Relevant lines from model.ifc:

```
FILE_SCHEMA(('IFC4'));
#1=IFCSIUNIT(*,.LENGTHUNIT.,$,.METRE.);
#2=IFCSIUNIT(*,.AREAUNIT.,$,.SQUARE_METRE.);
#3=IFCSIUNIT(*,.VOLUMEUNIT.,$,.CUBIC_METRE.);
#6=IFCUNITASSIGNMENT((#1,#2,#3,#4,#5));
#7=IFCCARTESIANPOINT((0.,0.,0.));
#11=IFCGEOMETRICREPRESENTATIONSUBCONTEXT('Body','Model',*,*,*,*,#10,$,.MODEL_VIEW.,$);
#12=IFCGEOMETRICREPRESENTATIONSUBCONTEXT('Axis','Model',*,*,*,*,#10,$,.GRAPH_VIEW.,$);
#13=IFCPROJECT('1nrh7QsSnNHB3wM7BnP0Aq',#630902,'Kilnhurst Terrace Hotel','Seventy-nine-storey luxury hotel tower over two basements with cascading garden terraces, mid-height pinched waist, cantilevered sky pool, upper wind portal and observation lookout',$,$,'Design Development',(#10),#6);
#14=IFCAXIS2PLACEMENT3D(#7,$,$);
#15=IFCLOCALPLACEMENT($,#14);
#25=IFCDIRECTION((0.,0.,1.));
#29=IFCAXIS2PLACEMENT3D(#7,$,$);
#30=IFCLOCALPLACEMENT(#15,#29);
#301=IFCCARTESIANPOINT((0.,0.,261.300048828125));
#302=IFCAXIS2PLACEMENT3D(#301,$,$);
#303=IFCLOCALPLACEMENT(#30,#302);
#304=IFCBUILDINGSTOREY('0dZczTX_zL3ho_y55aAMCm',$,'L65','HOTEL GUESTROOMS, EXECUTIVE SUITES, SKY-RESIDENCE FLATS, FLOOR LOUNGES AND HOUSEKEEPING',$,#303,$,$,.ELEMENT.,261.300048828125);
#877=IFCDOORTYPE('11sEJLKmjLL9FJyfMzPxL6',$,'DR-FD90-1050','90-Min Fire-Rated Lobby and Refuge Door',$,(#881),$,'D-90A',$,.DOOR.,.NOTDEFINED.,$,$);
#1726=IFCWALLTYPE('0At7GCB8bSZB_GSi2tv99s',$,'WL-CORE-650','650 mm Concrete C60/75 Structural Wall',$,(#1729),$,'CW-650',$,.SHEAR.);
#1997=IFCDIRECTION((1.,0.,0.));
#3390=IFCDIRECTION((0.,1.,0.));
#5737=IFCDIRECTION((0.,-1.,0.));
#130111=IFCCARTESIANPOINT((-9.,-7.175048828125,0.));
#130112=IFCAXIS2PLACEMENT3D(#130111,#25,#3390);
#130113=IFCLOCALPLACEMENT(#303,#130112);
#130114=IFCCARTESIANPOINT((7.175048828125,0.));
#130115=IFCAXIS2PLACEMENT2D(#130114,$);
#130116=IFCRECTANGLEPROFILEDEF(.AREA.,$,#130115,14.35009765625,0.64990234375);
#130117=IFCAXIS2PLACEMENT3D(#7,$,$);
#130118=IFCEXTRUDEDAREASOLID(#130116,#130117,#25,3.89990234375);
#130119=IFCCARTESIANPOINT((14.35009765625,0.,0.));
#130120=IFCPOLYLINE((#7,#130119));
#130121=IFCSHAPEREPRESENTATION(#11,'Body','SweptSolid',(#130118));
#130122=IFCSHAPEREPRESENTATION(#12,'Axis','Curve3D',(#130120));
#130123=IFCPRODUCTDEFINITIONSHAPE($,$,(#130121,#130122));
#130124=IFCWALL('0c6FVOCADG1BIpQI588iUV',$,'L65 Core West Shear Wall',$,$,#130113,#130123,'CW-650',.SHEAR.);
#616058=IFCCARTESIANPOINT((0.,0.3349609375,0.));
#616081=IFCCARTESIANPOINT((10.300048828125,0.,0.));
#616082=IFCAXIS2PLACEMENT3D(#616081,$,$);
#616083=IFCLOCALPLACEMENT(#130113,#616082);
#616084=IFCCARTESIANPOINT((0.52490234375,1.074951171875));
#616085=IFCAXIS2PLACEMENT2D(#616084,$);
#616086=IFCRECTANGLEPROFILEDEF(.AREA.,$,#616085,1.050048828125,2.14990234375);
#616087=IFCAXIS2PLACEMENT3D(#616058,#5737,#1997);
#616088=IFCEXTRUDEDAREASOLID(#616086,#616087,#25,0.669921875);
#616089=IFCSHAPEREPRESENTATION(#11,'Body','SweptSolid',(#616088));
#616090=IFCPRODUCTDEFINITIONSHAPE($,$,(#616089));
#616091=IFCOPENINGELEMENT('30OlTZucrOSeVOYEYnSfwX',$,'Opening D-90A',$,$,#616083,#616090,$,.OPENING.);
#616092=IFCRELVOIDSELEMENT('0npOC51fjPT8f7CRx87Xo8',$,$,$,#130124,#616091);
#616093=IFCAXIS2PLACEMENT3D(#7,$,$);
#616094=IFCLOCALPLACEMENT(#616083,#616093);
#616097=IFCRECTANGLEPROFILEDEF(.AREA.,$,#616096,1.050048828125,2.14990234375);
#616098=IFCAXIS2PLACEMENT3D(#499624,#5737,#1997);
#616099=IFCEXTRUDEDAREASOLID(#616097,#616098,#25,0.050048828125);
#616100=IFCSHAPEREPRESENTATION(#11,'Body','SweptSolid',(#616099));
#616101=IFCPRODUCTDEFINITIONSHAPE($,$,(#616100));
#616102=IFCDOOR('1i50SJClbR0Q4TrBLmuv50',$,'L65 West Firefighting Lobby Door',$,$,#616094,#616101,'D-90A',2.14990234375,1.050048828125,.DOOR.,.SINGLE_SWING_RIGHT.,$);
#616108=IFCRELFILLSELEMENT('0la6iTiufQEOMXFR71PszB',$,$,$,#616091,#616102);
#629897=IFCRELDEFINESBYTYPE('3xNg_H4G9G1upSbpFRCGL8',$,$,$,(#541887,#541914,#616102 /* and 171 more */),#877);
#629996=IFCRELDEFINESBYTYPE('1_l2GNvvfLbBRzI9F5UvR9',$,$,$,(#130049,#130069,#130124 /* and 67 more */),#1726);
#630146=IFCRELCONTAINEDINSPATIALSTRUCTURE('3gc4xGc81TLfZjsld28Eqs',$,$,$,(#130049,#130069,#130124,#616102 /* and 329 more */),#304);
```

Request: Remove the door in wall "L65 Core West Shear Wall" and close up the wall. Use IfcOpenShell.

```python
import ifcopenshell
import ifcopenshell.api.feature
import ifcopenshell.api.root
import ifcopenshell.geom
import ifcopenshell.util.shape

model = ifcopenshell.open("model.ifc")
settings = ifcopenshell.geom.settings()


def volume(element):
    """Net volume in cubic metres, openings subtracted."""
    shape = ifcopenshell.geom.create_shape(settings, element)
    return ifcopenshell.util.shape.get_volume(shape.geometry)


door = model.by_guid("1i50SJClbR0Q4TrBLmuv50")
opening = door.FillsVoids[0].RelatingOpeningElement
wall = opening.VoidsElements[0].RelatingBuildingElement
before = volume(wall)

ifcopenshell.api.root.remove_product(model, product=door)
ifcopenshell.api.feature.remove_feature(model, feature=opening)

after = volume(wall)

print(f"wall volume {before:.3f} -> {after:.3f} m3")

model.write("model_v2.ifc")
```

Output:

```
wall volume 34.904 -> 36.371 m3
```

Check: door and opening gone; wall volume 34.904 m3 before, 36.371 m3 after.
